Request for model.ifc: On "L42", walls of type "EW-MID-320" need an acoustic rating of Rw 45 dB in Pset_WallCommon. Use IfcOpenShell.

First a look at what the model holds.

```python
import ifcopenshell
import ifcopenshell.util.element

model = ifcopenshell.open("model.ifc")
print(model.schema)
storey = next(s for s in model.by_type("IfcBuildingStorey") if s.Name == "L42")
walls = [e for e in ifcopenshell.util.element.get_decomposition(storey) if e.is_a("IfcWall")]
seen = {}
for e in walls:
    element_type = ifcopenshell.util.element.get_type(e)
    key = (element_type.Name if element_type != e and element_type else None, ifcopenshell.util.element.get_pset(e, "Pset_WallCommon", "AcousticRating"))
    seen[key] = seen.get(key, 0) + 1
for (name, value), count in sorted(seen.items(), key=str):
    print(count, "x", name, "|", value)
```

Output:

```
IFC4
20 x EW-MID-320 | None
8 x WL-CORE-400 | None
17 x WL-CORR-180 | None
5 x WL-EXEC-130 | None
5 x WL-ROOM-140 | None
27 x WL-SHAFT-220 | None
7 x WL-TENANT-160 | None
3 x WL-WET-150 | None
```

```python
import ifcopenshell
import ifcopenshell.api.pset
import ifcopenshell.util.element

model = ifcopenshell.open("model.ifc")

storey = next(s for s in model.by_type("IfcBuildingStorey") if s.Name == "L42")
walls = [e for e in ifcopenshell.util.element.get_decomposition(storey) if e.is_a("IfcWall")]

count = 0
for e in walls:
    element_type = ifcopenshell.util.element.get_type(e)
    if element_type in (None, e) or element_type.Name != "EW-MID-320":
        continue
    found = ifcopenshell.util.element.get_pset(e, "Pset_WallCommon", should_inherit=False)
    if found:
        pset = model.by_id(found["id"])
        if len(ifcopenshell.util.element.get_elements_by_pset(pset)) > 1:
            pset = ifcopenshell.api.pset.unshare_pset(model, products=[e], pset=pset)[0]
    else:
        pset = ifcopenshell.api.pset.add_pset(model, product=e, name="Pset_WallCommon")
    ifcopenshell.api.pset.edit_pset(model, pset=pset, properties={"AcousticRating": "Rw 45 dB"})
    count += 1

print(count, "walls updated")

model.write("model-out.ifc")
```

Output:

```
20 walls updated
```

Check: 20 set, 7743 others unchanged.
